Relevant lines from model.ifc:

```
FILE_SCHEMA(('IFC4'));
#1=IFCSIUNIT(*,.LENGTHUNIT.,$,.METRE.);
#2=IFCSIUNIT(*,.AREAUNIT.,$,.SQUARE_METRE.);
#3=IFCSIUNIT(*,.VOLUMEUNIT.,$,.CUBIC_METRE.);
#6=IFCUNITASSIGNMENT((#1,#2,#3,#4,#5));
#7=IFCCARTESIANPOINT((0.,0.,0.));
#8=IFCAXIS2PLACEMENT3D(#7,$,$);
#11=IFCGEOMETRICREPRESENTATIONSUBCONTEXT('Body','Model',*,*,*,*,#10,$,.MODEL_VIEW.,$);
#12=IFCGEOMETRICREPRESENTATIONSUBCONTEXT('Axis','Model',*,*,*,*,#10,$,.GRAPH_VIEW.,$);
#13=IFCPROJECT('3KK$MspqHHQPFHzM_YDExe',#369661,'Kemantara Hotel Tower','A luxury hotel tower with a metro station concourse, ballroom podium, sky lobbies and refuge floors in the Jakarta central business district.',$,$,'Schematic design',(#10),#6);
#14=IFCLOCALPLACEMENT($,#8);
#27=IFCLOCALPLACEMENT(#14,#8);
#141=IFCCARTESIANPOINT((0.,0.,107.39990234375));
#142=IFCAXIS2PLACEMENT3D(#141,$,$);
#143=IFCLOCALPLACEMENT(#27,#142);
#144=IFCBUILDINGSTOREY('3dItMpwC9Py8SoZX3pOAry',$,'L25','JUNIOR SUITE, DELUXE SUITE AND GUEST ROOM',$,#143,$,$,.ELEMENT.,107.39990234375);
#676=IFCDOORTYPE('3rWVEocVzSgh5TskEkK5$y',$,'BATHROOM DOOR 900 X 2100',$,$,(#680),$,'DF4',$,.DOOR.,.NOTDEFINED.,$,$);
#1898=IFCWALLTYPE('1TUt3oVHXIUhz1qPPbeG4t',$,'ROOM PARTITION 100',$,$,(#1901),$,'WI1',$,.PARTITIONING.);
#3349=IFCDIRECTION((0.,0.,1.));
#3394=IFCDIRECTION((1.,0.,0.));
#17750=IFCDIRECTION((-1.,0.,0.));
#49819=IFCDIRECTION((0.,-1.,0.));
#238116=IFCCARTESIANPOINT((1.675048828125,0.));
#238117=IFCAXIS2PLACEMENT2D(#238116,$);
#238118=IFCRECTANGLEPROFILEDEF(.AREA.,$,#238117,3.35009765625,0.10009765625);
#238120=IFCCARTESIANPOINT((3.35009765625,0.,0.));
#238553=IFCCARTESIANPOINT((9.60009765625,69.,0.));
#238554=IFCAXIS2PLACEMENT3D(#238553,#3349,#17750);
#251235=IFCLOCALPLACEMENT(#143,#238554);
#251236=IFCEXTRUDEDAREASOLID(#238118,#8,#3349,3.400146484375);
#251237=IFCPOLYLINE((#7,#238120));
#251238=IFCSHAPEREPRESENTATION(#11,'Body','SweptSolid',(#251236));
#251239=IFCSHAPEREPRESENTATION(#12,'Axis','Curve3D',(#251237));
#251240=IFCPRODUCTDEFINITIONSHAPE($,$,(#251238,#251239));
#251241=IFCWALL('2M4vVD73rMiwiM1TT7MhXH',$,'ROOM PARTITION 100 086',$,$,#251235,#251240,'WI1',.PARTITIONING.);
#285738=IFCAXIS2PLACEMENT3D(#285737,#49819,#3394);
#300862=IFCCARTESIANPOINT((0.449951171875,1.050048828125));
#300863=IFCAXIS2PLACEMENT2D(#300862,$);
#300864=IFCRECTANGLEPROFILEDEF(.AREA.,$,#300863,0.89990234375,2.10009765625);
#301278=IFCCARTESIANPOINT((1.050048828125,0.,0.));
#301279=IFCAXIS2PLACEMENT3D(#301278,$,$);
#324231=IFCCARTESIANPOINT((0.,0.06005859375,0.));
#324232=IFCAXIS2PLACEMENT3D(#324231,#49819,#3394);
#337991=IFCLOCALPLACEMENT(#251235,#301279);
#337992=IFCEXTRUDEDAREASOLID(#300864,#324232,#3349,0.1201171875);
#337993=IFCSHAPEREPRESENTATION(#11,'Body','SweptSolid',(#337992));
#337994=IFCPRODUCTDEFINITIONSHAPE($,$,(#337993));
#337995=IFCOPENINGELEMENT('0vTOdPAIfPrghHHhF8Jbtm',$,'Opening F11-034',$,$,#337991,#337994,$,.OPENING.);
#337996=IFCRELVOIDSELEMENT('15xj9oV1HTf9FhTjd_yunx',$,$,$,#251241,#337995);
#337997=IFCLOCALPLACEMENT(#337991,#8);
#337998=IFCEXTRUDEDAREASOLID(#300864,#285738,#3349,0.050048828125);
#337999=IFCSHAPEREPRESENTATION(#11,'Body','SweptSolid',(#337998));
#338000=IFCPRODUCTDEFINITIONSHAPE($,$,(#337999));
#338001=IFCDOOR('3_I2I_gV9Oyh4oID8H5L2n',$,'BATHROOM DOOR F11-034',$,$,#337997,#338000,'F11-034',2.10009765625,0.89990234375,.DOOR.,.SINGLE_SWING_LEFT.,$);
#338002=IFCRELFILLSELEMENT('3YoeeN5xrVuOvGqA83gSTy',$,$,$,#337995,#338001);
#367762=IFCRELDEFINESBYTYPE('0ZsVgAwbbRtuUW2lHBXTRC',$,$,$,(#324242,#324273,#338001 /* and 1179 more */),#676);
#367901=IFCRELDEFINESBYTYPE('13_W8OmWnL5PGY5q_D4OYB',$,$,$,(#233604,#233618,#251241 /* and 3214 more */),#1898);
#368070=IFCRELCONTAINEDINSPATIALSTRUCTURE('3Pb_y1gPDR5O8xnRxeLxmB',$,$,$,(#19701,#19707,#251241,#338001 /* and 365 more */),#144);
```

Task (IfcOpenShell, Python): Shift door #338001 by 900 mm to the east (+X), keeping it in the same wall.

```python
import ifcopenshell
import ifcopenshell.api.geometry
import ifcopenshell.util.placement

model = ifcopenshell.open("model.ifc")

door = model.by_guid("3_I2I_gV9Oyh4oID8H5L2n")
opening = door.FillsVoids[0].RelatingOpeningElement
wall = opening.VoidsElements[0].RelatingBuildingElement

wall_matrix = ifcopenshell.util.placement.get_local_placement(wall.ObjectPlacement)
shift = wall_matrix[:3, 0] * -0.9
before = ifcopenshell.util.placement.get_local_placement(door.ObjectPlacement)[:3, 3].copy()

# The door is placed relative to its opening, so it follows when the opening moves.
matrix = ifcopenshell.util.placement.get_local_placement(opening.ObjectPlacement)
matrix[:3, 3] += shift
ifcopenshell.api.geometry.edit_object_placement(
    model, product=opening, matrix=matrix, is_si=False, should_transform_children=True
)

after = ifcopenshell.util.placement.get_local_placement(door.ObjectPlacement)[:3, 3]
print("door moved by", (after - before).round(3) + 0.0)

model.write("model_edited.ifc")
```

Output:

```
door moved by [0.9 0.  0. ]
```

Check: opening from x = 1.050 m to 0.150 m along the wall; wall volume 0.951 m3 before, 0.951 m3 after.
